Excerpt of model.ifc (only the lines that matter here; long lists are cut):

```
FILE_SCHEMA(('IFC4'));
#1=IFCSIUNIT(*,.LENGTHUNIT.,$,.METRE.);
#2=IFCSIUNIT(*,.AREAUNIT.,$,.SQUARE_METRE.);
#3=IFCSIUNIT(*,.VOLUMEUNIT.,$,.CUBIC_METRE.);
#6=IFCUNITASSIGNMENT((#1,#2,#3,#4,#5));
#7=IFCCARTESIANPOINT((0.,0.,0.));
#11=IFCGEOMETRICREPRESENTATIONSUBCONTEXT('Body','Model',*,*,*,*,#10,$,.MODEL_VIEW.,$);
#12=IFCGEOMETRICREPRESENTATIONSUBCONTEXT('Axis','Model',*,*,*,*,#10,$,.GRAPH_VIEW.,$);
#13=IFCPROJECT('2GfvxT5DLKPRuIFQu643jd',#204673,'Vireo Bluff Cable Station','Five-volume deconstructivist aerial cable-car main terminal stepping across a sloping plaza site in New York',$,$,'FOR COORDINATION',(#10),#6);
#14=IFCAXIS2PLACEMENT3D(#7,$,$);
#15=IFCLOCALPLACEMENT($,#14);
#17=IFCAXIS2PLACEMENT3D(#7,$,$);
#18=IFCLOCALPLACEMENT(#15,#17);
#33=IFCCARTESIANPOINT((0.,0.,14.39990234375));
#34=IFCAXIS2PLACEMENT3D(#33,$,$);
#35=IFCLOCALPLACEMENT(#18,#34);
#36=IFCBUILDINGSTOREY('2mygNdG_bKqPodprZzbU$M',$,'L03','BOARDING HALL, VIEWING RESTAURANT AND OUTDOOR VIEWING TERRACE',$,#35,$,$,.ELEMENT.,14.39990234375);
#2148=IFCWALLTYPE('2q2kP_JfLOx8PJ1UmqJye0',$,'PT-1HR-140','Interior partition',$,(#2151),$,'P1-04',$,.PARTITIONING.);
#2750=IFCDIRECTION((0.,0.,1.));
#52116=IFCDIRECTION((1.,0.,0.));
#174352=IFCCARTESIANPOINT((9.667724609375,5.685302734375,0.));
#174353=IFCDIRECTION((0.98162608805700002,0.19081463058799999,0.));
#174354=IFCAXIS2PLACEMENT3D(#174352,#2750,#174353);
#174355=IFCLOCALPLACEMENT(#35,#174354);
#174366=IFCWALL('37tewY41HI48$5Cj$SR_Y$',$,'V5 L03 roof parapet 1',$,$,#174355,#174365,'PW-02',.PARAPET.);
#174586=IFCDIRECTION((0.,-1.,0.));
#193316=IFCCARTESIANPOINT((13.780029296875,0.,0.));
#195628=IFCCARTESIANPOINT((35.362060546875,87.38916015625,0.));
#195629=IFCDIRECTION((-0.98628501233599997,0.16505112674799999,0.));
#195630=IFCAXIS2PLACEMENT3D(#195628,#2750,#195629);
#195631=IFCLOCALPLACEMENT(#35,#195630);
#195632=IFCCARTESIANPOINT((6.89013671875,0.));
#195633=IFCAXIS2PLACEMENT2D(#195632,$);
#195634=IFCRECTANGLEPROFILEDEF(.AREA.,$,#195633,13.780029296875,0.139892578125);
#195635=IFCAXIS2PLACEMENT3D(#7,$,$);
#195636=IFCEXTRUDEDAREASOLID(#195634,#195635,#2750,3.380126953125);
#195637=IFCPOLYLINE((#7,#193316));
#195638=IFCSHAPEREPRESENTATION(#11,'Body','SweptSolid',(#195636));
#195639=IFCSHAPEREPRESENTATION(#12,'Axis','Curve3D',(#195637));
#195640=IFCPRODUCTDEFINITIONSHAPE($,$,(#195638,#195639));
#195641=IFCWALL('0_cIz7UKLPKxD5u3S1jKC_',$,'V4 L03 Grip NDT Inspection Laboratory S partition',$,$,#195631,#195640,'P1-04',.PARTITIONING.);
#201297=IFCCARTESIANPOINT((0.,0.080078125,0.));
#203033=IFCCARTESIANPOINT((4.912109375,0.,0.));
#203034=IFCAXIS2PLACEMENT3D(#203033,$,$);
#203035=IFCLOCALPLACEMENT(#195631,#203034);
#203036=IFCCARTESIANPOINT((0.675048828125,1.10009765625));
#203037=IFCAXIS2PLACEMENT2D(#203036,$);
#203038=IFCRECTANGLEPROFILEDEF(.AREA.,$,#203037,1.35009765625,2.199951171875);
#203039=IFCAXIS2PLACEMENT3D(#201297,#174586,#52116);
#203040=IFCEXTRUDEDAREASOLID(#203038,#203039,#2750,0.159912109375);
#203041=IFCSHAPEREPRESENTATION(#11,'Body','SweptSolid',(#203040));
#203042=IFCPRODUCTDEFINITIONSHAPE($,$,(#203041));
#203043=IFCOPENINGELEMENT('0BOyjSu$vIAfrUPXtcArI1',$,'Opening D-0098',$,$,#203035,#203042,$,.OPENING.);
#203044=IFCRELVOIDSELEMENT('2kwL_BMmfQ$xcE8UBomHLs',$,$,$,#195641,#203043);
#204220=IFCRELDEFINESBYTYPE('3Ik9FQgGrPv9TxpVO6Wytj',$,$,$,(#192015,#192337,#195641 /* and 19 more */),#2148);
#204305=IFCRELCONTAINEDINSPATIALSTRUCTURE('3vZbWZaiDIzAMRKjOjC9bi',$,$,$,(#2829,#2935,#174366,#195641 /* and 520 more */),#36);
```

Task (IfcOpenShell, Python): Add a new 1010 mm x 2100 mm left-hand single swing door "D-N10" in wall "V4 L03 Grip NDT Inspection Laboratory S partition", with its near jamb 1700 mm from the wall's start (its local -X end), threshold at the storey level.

```python
import numpy as np
import ifcopenshell
import ifcopenshell.api.feature
import ifcopenshell.api.geometry
import ifcopenshell.api.root
import ifcopenshell.api.spatial
import ifcopenshell.geom
import ifcopenshell.util.element
import ifcopenshell.util.placement
import ifcopenshell.util.representation
import ifcopenshell.util.shape
import ifcopenshell.util.unit

model = ifcopenshell.open("model.ifc")
unit_scale = ifcopenshell.util.unit.calculate_unit_scale(model)
settings = ifcopenshell.geom.settings()


def volume(element):
    """Net volume in cubic metres, openings subtracted."""
    shape = ifcopenshell.geom.create_shape(settings, element)
    return ifcopenshell.util.shape.get_volume(shape.geometry)


wall = model.by_guid("0_cIz7UKLPKxD5u3S1jKC_")
storey = ifcopenshell.util.element.get_container(wall, ifc_class="IfcBuildingStorey")
context = ifcopenshell.util.representation.get_context(model, "Model", "Body", "MODEL_VIEW")
before = volume(wall)

width, height, from_end, sill = 1.01, 2.1, 1.7, 0.0  # metres

# The wall runs along its own X axis, and the end named is its -X end.
wall_shape = ifcopenshell.geom.create_shape(settings, wall)
x, y, z = ifcopenshell.util.shape.get_vertices(wall_shape.geometry).T
start = x.min() + from_end
face, thickness = float(y.min()), float(y.max() - y.min())
wall_matrix = ifcopenshell.util.placement.get_local_placement(wall.ObjectPlacement)
level = ifcopenshell.util.placement.get_local_placement(storey.ObjectPlacement)[2, 3]


def in_wall(x, y):
    """Placement at x, y metres in the wall's axes, at sill height."""
    matrix = wall_matrix.copy()
    matrix[:, 3] = wall_matrix @ np.array([x / unit_scale, y / unit_scale, 0.0, 1.0])
    matrix[2, 3] = level + sill / unit_scale
    return matrix


# Opening: a box that overshoots both wall faces by 50 mm.
opening = ifcopenshell.api.root.create_entity(model, ifc_class="IfcOpeningElement", predefined_type="OPENING")
box = ifcopenshell.api.geometry.add_wall_representation(
    model, context=context, length=width, height=height, thickness=thickness + 0.1
)
ifcopenshell.api.geometry.assign_representation(model, product=opening, representation=box)
ifcopenshell.api.geometry.edit_object_placement(model, product=opening, matrix=in_wall(start, face - 0.05), is_si=False)
ifcopenshell.api.feature.add_feature(model, feature=opening, element=wall)

door = ifcopenshell.api.root.create_entity(model, ifc_class="IfcDoor", name="D-N10", predefined_type="DOOR")
door.OverallWidth, door.OverallHeight = width / unit_scale, height / unit_scale
door.OperationType = "SINGLE_SWING_LEFT"
body = ifcopenshell.api.geometry.add_door_representation(
    model,
    context=context,
    overall_width=door.OverallWidth,
    overall_height=door.OverallHeight,
    operation_type="SINGLE_SWING_LEFT",
    lining_properties={"LiningDepth": thickness / unit_scale, "ThresholdDepth": thickness / unit_scale},
)
ifcopenshell.api.geometry.assign_representation(model, product=door, representation=body)
ifcopenshell.api.spatial.assign_container(model, products=[door], relating_structure=storey)
ifcopenshell.api.feature.add_filling(model, opening=opening, element=door)

# The lining spans the wall, so the door starts at the wall face.
ifcopenshell.api.geometry.edit_object_placement(model, product=door, matrix=in_wall(start, face), is_si=False)

after = volume(wall)

print(f"wall volume {before:.3f} -> {after:.3f} m3")

model.write("model_edited.ifc")
```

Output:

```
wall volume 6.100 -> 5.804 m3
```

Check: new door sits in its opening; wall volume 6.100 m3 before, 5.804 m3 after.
